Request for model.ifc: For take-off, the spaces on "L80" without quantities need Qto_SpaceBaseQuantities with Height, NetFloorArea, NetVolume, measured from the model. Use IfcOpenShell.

First a look at what the model holds.

```python
import ifcopenshell
import ifcopenshell.util.element
import ifcopenshell.util.unit

model = ifcopenshell.open("model.ifc")
print(model.schema)
for unit_type in ("LENGTHUNIT", "AREAUNIT", "VOLUMEUNIT"):
    print(unit_type, ifcopenshell.util.unit.calculate_unit_scale(model, unit_type))
storey = next(s for s in model.by_type("IfcBuildingStorey") if s.Name == "L80")
spaces = [e for e in ifcopenshell.util.element.get_decomposition(storey) if e.is_a("IfcSpace")]
for e in sorted(spaces, key=lambda e: e.id()):
    print(e.id(), e.is_a(), e.Name, list(ifcopenshell.util.element.get_psets(e, qtos_only=True)), sep=" | ")
```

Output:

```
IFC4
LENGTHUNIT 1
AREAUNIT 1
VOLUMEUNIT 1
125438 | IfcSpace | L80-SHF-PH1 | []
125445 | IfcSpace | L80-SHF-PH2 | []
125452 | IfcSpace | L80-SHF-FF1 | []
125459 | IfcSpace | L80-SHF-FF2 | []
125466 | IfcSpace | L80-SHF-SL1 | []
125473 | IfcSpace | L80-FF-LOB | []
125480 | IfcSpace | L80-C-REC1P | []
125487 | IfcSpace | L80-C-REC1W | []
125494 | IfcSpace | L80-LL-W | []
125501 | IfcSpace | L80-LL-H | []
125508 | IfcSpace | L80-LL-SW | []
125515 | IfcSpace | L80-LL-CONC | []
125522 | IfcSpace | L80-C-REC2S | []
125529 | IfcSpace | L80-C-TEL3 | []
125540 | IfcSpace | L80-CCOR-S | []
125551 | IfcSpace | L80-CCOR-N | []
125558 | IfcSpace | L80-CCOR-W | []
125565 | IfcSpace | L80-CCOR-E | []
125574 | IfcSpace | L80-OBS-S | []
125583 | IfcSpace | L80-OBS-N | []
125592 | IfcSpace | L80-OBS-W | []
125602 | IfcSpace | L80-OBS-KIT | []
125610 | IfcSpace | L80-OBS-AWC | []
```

```python
import ifcopenshell
import ifcopenshell.api.pset
import ifcopenshell.geom
import ifcopenshell.util.element
import ifcopenshell.util.shape
import ifcopenshell.util.unit

model = ifcopenshell.open("model.ifc")
unit_scale = ifcopenshell.util.unit.calculate_unit_scale(model)
area_scale = ifcopenshell.util.unit.calculate_unit_scale(model, "AREAUNIT")
volume_scale = ifcopenshell.util.unit.calculate_unit_scale(model, "VOLUMEUNIT")
settings = ifcopenshell.geom.settings()

storey = next(s for s in model.by_type("IfcBuildingStorey") if s.Name == "L80")
spaces = [e for e in ifcopenshell.util.element.get_decomposition(storey) if e.is_a("IfcSpace")]

for e in sorted(spaces, key=lambda e: e.id()):
    if ifcopenshell.util.element.get_psets(e, qtos_only=True, should_inherit=False):
        continue
    # Geometry comes back in metres, in the element's own axes.
    shape = ifcopenshell.geom.create_shape(settings, e)
    values = {
        "Height": ifcopenshell.util.shape.get_z(shape.geometry) / unit_scale,
        "NetFloorArea": ifcopenshell.util.shape.get_footprint_area(shape.geometry) / area_scale,
        "NetVolume": ifcopenshell.util.shape.get_volume(shape.geometry) / volume_scale,
    }
    qto = ifcopenshell.api.pset.add_qto(model, product=e, name="Qto_SpaceBaseQuantities")
    ifcopenshell.api.pset.edit_qto(model, qto=qto, properties=values)
    print(e.id(), {k: round(v, 3) for k, v in values.items()})

model.write("model_edited.ifc")
```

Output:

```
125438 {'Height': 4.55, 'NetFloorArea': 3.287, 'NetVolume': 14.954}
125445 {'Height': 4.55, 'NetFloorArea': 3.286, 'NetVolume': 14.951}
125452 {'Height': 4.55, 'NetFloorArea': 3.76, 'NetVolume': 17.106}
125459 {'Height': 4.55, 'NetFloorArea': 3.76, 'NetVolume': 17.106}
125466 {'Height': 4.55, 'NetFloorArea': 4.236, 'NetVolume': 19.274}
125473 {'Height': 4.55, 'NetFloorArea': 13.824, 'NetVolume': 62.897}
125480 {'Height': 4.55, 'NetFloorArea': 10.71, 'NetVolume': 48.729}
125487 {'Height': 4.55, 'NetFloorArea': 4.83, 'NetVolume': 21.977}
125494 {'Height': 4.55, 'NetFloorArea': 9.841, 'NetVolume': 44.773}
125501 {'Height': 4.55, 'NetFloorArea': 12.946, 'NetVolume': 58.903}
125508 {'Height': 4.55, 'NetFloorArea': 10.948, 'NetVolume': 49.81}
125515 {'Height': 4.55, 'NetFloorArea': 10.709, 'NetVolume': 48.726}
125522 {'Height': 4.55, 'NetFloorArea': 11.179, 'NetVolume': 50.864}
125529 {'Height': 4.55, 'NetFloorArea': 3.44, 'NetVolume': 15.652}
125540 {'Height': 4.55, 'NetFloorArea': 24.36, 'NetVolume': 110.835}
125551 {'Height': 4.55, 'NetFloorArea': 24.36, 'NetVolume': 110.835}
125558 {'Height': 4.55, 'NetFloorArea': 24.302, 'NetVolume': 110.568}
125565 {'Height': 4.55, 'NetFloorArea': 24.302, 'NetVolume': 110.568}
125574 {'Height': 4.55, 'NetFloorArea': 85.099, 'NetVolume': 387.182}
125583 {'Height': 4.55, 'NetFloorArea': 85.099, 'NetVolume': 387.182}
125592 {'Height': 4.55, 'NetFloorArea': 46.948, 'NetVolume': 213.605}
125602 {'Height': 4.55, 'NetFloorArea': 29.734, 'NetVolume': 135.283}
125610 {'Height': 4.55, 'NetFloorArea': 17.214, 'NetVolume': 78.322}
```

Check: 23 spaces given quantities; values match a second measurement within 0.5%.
